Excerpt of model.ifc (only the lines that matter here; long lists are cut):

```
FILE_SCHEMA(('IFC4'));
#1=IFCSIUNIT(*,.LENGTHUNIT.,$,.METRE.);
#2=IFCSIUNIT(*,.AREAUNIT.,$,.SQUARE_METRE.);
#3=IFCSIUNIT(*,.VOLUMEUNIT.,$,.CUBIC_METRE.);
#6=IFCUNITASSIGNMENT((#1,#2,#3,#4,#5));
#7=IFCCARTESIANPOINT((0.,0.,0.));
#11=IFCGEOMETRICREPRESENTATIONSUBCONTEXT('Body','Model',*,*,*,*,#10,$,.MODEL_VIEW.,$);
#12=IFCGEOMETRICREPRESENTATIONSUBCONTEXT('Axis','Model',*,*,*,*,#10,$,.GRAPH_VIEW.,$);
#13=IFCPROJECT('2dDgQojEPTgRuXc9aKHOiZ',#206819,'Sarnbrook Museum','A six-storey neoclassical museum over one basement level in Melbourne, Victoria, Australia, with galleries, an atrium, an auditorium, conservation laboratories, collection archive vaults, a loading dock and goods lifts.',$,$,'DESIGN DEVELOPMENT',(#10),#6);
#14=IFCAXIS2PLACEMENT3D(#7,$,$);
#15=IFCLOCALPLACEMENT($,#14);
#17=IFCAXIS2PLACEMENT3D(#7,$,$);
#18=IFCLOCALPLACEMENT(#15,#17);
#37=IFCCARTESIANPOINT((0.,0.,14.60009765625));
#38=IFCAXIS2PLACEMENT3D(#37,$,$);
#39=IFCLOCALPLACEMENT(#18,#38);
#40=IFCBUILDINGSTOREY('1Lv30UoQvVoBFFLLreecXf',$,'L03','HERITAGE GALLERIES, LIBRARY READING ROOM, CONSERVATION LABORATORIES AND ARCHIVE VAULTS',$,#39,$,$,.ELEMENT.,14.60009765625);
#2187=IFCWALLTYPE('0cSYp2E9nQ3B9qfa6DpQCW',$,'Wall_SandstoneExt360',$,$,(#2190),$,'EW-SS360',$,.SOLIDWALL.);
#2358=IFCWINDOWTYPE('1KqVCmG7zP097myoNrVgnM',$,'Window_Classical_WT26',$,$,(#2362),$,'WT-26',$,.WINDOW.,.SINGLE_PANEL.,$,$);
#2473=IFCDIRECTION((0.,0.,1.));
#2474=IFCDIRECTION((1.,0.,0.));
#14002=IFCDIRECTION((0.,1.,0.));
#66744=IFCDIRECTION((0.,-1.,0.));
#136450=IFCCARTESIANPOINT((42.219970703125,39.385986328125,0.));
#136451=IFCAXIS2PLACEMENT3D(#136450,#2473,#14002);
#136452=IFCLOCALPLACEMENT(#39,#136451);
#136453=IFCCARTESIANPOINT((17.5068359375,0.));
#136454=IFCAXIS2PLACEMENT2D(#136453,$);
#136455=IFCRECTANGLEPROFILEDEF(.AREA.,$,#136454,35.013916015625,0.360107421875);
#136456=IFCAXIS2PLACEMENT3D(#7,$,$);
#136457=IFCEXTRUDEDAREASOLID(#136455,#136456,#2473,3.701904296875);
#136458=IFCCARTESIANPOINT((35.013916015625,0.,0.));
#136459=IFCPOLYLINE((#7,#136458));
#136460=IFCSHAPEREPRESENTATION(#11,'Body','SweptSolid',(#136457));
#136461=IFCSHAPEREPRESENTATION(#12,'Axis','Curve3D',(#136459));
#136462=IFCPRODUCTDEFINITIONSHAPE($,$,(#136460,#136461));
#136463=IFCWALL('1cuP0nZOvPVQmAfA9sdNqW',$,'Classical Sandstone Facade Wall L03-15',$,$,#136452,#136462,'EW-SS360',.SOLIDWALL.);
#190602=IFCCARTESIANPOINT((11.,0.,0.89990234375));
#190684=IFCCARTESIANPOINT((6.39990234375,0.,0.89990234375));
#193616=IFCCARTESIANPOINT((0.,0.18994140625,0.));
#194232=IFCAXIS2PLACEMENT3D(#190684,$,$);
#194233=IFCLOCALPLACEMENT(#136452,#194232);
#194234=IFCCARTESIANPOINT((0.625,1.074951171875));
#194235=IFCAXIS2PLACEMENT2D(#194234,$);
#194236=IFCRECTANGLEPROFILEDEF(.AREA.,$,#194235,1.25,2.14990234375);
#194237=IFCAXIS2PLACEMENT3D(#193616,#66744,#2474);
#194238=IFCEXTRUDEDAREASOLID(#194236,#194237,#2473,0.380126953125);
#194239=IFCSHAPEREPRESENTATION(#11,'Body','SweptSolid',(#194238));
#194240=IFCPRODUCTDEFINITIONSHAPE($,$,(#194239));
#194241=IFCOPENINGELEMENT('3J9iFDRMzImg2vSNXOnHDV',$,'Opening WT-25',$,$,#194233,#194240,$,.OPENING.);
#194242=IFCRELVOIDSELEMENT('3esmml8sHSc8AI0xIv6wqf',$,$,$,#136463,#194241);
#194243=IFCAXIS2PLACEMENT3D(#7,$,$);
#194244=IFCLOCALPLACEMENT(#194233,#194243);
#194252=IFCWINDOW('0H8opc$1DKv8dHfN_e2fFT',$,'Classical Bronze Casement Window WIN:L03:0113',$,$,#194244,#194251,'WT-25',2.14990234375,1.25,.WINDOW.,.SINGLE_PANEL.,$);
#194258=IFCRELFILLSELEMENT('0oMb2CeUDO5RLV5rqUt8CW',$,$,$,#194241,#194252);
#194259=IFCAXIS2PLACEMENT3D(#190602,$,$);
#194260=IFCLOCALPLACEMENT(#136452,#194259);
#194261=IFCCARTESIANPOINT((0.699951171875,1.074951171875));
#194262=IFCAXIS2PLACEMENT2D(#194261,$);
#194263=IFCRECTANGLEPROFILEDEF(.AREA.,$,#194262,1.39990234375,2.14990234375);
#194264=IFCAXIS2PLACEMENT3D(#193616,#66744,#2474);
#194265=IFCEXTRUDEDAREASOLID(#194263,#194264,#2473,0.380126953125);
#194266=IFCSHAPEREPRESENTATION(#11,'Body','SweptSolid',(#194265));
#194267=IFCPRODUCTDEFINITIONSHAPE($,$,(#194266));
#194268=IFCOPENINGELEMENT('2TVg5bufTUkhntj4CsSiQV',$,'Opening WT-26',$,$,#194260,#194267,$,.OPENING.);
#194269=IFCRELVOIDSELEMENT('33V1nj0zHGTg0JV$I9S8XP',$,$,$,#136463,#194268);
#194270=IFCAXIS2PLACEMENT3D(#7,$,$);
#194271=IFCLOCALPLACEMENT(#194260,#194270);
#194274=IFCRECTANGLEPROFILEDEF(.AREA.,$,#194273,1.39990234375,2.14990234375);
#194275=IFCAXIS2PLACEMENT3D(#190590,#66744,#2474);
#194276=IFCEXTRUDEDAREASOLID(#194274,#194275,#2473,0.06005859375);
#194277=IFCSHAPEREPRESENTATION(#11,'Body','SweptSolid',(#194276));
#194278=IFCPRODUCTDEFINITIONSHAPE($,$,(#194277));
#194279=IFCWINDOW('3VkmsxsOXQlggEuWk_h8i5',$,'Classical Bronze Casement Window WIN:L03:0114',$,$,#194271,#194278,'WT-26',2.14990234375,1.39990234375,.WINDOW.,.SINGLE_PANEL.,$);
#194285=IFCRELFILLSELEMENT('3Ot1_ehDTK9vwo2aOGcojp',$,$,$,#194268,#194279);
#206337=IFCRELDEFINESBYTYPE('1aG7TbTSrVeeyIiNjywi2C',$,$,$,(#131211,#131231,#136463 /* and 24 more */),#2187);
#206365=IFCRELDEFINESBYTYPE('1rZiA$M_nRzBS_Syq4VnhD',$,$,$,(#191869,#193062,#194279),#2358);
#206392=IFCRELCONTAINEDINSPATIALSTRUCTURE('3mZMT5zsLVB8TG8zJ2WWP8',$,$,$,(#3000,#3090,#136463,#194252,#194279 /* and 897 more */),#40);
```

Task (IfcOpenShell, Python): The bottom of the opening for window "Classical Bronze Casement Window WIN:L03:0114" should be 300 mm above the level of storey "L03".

```python
import numpy as np
import ifcopenshell
import ifcopenshell.api.geometry
import ifcopenshell.geom
import ifcopenshell.util.element
import ifcopenshell.util.placement
import ifcopenshell.util.shape
import ifcopenshell.util.unit

model = ifcopenshell.open("model.ifc")
unit_scale = ifcopenshell.util.unit.calculate_unit_scale(model)

window = model.by_id(194279)
opening = window.FillsVoids[0].RelatingOpeningElement
storey = ifcopenshell.util.element.get_container(window, ifc_class="IfcBuildingStorey")
level = ifcopenshell.util.placement.get_local_placement(storey.ObjectPlacement)[2, 3]

# The opening's origin need not be at the sill, so measure its lowest point.
shape = ifcopenshell.geom.create_shape(ifcopenshell.geom.settings(), opening)
bottom = ifcopenshell.util.shape.get_shape_bottom_elevation(shape, shape.geometry) / unit_scale
dz = level + 0.3 / unit_scale - bottom

shift = np.array([0.0, 0.0, dz])
# The window is placed relative to its opening, so it follows when the opening moves.
matrix = ifcopenshell.util.placement.get_local_placement(opening.ObjectPlacement)
matrix[:3, 3] += shift
ifcopenshell.api.geometry.edit_object_placement(
    model, product=opening, matrix=matrix, is_si=False, should_transform_children=True
)

print(f"moved by {dz * unit_scale:+.3f} m")

model.write("model_edited.ifc")
```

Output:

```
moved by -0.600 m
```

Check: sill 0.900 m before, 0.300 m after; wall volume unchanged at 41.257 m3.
